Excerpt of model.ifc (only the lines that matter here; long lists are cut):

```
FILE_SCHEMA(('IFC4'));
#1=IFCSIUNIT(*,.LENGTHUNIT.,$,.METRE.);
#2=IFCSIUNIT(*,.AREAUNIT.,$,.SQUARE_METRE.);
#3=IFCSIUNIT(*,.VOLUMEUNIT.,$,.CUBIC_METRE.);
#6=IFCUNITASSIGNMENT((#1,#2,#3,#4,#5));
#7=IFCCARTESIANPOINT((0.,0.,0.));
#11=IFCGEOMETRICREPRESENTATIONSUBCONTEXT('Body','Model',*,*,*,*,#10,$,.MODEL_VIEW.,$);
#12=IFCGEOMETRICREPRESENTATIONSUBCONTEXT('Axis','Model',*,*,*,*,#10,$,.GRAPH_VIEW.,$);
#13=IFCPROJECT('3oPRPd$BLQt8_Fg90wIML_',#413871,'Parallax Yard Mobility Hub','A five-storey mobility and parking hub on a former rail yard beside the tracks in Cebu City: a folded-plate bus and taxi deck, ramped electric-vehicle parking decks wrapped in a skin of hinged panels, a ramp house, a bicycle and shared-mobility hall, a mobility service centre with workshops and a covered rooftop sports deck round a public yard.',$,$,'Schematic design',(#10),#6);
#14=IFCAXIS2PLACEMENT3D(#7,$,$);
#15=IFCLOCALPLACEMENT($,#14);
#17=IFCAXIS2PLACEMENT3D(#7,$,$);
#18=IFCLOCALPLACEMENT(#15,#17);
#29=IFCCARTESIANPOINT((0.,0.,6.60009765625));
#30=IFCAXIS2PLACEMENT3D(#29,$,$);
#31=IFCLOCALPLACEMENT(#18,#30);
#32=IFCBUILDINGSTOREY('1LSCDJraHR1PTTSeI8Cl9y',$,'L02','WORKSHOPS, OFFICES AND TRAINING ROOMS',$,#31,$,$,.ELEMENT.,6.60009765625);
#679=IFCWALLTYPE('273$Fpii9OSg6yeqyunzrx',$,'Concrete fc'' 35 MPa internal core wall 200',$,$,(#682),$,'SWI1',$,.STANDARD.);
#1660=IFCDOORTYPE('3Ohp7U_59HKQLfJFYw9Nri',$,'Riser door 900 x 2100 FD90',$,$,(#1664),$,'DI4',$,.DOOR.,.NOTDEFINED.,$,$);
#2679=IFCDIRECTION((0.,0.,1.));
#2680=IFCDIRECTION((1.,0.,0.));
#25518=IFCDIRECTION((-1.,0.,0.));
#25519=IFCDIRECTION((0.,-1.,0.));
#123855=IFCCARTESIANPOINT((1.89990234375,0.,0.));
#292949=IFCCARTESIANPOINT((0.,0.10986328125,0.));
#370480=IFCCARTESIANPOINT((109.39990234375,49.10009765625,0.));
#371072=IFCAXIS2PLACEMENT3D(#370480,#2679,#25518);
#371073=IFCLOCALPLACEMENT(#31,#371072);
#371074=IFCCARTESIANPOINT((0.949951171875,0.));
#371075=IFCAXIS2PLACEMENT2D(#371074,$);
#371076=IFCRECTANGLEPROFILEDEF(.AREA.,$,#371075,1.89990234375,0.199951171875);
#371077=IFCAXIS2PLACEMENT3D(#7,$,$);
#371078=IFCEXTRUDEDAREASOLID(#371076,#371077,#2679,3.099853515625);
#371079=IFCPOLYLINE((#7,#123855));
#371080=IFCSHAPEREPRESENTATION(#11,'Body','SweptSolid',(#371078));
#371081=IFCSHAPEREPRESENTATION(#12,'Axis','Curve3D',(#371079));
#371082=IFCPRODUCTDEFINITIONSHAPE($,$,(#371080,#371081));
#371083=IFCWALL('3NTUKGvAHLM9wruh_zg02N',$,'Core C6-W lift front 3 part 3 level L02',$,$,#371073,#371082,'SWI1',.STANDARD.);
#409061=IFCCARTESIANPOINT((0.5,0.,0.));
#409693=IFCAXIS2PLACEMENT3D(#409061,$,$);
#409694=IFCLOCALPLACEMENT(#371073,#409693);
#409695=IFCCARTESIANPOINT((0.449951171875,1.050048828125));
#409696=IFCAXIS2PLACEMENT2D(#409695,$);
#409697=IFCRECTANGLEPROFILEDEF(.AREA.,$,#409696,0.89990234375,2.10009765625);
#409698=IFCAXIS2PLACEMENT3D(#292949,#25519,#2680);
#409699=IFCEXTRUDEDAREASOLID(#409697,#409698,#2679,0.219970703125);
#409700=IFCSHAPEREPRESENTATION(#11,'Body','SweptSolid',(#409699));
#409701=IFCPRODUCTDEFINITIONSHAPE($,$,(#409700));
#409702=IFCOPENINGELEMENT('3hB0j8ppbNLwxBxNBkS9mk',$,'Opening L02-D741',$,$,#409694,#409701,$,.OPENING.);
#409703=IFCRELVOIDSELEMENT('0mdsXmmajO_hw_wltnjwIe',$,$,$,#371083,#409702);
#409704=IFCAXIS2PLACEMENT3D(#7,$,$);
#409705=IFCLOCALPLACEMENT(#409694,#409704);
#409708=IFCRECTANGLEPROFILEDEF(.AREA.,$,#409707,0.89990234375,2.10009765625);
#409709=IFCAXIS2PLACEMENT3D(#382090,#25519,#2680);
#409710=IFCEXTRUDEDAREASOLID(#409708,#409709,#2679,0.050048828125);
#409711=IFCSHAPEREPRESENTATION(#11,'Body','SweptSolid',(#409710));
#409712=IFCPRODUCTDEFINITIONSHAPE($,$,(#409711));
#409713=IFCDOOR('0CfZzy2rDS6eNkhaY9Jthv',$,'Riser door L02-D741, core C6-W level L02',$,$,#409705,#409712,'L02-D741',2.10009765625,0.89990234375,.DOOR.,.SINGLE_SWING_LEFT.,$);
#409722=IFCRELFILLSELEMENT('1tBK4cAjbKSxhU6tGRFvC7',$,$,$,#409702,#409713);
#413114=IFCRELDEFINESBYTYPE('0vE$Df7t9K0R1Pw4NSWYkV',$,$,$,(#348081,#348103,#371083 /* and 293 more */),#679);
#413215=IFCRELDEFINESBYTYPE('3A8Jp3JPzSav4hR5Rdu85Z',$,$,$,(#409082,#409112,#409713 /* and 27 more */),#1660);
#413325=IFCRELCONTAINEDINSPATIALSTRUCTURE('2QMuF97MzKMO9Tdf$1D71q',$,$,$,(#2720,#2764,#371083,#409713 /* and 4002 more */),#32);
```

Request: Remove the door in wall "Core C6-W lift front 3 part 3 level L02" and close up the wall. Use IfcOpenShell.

```python
import ifcopenshell
import ifcopenshell.api.feature
import ifcopenshell.api.root
import ifcopenshell.geom
import ifcopenshell.util.shape

model = ifcopenshell.open("model.ifc")
settings = ifcopenshell.geom.settings()


def volume(element):
    """Net volume in cubic metres, openings subtracted."""
    shape = ifcopenshell.geom.create_shape(settings, element)
    return ifcopenshell.util.shape.get_volume(shape.geometry)


door = model.by_guid("0CfZzy2rDS6eNkhaY9Jthv")
opening = door.FillsVoids[0].RelatingOpeningElement
wall = opening.VoidsElements[0].RelatingBuildingElement
before = volume(wall)

ifcopenshell.api.root.remove_product(model, product=door)
ifcopenshell.api.feature.remove_feature(model, feature=opening)

after = volume(wall)

print(f"wall volume {before:.3f} -> {after:.3f} m3")

model.write("model_updated.ifc")
```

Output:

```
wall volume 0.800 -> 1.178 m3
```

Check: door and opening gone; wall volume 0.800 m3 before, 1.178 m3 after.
